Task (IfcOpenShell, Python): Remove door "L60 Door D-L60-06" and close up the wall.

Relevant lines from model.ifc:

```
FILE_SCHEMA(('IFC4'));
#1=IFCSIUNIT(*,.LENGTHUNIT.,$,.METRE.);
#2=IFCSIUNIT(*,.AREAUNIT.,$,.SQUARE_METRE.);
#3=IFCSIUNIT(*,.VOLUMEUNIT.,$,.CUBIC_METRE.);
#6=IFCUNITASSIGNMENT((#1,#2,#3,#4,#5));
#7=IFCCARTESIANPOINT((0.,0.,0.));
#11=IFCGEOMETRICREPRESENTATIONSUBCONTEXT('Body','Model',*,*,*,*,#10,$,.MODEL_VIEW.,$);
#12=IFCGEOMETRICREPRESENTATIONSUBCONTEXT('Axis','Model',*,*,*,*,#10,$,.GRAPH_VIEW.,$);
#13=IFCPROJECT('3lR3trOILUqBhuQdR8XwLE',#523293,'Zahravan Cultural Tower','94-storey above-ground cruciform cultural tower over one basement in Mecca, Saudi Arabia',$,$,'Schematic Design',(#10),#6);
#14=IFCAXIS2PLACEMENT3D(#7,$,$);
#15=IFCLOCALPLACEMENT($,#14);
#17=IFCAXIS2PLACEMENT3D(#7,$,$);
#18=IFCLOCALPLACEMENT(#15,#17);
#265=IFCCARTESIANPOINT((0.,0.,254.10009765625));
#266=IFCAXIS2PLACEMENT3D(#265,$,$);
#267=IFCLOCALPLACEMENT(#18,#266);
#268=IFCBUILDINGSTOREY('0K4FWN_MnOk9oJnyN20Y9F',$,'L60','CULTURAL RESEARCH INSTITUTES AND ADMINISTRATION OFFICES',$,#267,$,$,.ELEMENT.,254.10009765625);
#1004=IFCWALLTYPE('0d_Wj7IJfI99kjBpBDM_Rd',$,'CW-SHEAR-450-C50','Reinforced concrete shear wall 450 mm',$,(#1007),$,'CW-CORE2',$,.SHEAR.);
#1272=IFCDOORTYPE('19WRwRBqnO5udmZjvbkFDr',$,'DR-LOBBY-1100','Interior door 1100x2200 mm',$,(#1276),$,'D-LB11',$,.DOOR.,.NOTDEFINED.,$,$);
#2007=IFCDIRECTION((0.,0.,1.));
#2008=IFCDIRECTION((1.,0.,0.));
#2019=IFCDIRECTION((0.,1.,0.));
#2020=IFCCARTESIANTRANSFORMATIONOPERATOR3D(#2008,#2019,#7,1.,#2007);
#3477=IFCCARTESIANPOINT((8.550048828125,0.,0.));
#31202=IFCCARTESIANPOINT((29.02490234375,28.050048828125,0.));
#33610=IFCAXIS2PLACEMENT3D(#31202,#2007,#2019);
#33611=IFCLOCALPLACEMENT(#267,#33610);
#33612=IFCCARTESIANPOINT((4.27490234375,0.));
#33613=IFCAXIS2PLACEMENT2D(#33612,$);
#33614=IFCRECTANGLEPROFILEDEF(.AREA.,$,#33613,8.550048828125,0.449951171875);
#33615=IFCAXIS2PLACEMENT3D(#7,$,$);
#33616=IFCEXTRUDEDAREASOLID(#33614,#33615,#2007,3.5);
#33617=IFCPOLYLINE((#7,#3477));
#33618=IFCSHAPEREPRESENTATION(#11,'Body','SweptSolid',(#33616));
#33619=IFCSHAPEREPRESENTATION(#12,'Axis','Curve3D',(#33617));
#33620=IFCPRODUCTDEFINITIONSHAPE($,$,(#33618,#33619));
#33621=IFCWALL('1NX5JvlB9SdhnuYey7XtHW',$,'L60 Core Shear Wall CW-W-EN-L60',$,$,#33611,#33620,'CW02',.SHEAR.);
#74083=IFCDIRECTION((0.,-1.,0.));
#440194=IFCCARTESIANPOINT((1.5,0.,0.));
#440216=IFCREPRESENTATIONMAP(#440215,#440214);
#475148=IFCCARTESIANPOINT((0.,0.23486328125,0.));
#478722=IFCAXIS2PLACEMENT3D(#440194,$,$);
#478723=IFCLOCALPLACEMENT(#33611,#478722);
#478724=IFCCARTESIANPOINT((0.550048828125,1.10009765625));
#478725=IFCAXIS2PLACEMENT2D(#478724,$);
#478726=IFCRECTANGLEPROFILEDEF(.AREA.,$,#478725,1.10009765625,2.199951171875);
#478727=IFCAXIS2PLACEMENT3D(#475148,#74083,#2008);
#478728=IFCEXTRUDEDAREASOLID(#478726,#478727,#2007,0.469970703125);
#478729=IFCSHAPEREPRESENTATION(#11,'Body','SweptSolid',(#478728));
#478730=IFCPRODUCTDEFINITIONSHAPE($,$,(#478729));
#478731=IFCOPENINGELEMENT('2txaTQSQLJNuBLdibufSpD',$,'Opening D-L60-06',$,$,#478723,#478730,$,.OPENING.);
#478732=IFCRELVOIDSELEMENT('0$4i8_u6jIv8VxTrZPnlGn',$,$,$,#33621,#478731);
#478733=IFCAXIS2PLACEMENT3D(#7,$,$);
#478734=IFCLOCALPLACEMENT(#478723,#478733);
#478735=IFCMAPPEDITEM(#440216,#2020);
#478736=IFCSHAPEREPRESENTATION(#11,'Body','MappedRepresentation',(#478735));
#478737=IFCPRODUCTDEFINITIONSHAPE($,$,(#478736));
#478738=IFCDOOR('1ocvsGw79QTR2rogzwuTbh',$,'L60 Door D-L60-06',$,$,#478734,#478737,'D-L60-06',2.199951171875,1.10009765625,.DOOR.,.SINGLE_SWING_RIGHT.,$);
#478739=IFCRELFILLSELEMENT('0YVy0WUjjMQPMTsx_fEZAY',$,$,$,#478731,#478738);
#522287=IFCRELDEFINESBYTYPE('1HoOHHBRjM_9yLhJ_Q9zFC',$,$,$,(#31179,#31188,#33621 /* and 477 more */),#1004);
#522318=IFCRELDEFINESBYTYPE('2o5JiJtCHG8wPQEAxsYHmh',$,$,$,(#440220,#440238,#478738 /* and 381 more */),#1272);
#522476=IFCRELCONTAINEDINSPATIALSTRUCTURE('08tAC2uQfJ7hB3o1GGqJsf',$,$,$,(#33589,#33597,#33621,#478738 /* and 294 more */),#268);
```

```python
import ifcopenshell
import ifcopenshell.api.feature
import ifcopenshell.api.root
import ifcopenshell.geom
import ifcopenshell.util.shape

model = ifcopenshell.open("model.ifc")
settings = ifcopenshell.geom.settings()


def volume(element):
    """Net volume in cubic metres, openings subtracted."""
    shape = ifcopenshell.geom.create_shape(settings, element)
    return ifcopenshell.util.shape.get_volume(shape.geometry)


door = model.by_guid("1ocvsGw79QTR2rogzwuTbh")
opening = door.FillsVoids[0].RelatingOpeningElement
wall = opening.VoidsElements[0].RelatingBuildingElement
before = volume(wall)

ifcopenshell.api.root.remove_product(model, product=door)
ifcopenshell.api.feature.remove_feature(model, feature=opening)

after = volume(wall)

print(f"wall volume {before:.3f} -> {after:.3f} m3")

model.write("model_rev.ifc")
```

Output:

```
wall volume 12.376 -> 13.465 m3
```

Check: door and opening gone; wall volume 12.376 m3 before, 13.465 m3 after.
